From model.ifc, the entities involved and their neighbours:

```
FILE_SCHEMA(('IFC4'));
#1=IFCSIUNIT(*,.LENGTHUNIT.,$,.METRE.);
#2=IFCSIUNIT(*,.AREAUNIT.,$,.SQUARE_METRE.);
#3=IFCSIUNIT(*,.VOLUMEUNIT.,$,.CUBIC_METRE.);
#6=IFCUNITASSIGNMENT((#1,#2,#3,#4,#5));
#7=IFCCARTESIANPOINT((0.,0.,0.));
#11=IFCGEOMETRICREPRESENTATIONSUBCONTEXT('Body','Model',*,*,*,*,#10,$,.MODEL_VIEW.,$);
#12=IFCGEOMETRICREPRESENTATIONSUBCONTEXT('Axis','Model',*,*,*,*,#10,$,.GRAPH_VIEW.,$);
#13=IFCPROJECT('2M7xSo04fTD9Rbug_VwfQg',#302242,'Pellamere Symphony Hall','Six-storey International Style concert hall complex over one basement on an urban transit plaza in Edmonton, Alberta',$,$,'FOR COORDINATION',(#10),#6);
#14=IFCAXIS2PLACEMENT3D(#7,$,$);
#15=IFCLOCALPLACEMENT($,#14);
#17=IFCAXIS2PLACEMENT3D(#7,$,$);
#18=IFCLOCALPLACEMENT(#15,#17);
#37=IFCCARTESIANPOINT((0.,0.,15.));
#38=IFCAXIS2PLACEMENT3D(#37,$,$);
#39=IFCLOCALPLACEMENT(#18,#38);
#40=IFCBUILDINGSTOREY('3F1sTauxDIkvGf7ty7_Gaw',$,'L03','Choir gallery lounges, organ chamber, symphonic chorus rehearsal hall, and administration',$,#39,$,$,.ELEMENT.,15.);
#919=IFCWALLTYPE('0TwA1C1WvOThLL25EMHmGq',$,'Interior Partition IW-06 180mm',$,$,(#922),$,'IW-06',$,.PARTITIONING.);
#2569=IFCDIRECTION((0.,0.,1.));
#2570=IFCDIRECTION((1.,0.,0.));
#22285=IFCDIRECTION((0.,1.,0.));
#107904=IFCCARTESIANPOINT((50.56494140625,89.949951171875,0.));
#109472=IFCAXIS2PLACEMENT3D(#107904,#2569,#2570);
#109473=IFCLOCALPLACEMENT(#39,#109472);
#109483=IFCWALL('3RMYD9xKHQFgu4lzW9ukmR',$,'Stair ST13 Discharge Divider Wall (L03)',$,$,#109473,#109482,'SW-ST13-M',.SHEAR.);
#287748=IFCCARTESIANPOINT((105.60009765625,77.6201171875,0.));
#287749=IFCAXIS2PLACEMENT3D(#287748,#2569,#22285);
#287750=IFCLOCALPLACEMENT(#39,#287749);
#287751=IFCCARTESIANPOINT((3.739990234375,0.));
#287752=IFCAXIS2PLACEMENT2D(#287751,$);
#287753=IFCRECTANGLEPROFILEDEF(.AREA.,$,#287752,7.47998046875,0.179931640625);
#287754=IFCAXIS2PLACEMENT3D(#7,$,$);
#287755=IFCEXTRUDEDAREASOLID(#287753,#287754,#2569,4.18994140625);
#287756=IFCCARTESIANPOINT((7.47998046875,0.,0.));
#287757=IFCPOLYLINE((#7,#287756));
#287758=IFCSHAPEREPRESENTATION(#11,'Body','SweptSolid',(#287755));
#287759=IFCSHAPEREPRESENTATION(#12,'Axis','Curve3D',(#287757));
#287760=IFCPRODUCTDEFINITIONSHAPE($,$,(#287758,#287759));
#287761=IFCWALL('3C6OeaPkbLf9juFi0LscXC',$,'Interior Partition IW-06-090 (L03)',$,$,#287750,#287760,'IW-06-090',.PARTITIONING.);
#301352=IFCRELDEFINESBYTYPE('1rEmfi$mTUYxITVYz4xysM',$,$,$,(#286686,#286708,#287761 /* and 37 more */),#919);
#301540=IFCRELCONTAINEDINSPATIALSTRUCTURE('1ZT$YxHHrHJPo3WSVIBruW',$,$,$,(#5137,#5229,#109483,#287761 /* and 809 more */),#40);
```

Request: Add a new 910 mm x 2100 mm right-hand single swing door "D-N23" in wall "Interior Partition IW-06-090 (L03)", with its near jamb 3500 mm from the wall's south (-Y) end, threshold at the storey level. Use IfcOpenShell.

```python
import numpy as np
import ifcopenshell
import ifcopenshell.api.feature
import ifcopenshell.api.geometry
import ifcopenshell.api.root
import ifcopenshell.api.spatial
import ifcopenshell.geom
import ifcopenshell.util.element
import ifcopenshell.util.placement
import ifcopenshell.util.representation
import ifcopenshell.util.shape
import ifcopenshell.util.unit

model = ifcopenshell.open("model.ifc")
unit_scale = ifcopenshell.util.unit.calculate_unit_scale(model)
settings = ifcopenshell.geom.settings()


def volume(element):
    """Net volume in cubic metres, openings subtracted."""
    shape = ifcopenshell.geom.create_shape(settings, element)
    return ifcopenshell.util.shape.get_volume(shape.geometry)


wall = model.by_id(287761)
storey = ifcopenshell.util.element.get_container(wall, ifc_class="IfcBuildingStorey")
context = ifcopenshell.util.representation.get_context(model, "Model", "Body", "MODEL_VIEW")
before = volume(wall)

width, height, from_end, sill = 0.91, 2.1, 3.5, 0.0  # metres

# The wall runs along its own X axis, and the end named is its -X end.
wall_shape = ifcopenshell.geom.create_shape(settings, wall)
x, y, z = ifcopenshell.util.shape.get_vertices(wall_shape.geometry).T
start = x.min() + from_end
face, thickness = float(y.min()), float(y.max() - y.min())
wall_matrix = ifcopenshell.util.placement.get_local_placement(wall.ObjectPlacement)
level = ifcopenshell.util.placement.get_local_placement(storey.ObjectPlacement)[2, 3]


def in_wall(x, y):
    """Placement at x, y metres in the wall's axes, at sill height."""
    matrix = wall_matrix.copy()
    matrix[:, 3] = wall_matrix @ np.array([x / unit_scale, y / unit_scale, 0.0, 1.0])
    matrix[2, 3] = level + sill / unit_scale
    return matrix


# Opening: a box that overshoots both wall faces by 50 mm.
opening = ifcopenshell.api.root.create_entity(model, ifc_class="IfcOpeningElement", predefined_type="OPENING")
box = ifcopenshell.api.geometry.add_wall_representation(
    model, context=context, length=width, height=height, thickness=thickness + 0.1
)
ifcopenshell.api.geometry.assign_representation(model, product=opening, representation=box)
ifcopenshell.api.geometry.edit_object_placement(model, product=opening, matrix=in_wall(start, face - 0.05), is_si=False)
ifcopenshell.api.feature.add_feature(model, feature=opening, element=wall)

door = ifcopenshell.api.root.create_entity(model, ifc_class="IfcDoor", name="D-N23", predefined_type="DOOR")
door.OverallWidth, door.OverallHeight = width / unit_scale, height / unit_scale
door.OperationType = "SINGLE_SWING_RIGHT"
body = ifcopenshell.api.geometry.add_door_representation(
    model,
    context=context,
    overall_width=door.OverallWidth,
    overall_height=door.OverallHeight,
    operation_type="SINGLE_SWING_RIGHT",
    lining_properties={"LiningDepth": thickness / unit_scale, "ThresholdDepth": thickness / unit_scale},
)
ifcopenshell.api.geometry.assign_representation(model, product=door, representation=body)
ifcopenshell.api.spatial.assign_container(model, products=[door], relating_structure=storey)
ifcopenshell.api.feature.add_filling(model, opening=opening, element=door)

# The lining spans the wall, so the door starts at the wall face.
ifcopenshell.api.geometry.edit_object_placement(model, product=door, matrix=in_wall(start, face), is_si=False)

after = volume(wall)

print(f"wall volume {before:.3f} -> {after:.3f} m3")

model.write("model_updated.ifc")
```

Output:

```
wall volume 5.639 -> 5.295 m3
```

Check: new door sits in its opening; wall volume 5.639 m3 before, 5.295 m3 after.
